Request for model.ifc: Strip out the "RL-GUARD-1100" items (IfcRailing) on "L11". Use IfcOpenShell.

First a look at what the model holds.

```python
import ifcopenshell
import ifcopenshell.util.element

model = ifcopenshell.open("model.ifc")
print(model.schema)
storey = next(s for s in model.by_type("IfcBuildingStorey") if s.Name == "L11")
railings = [e for e in ifcopenshell.util.element.get_decomposition(storey) if e.is_a("IfcRailing")]
seen = {}
for e in railings:
    element_type = ifcopenshell.util.element.get_type(e)
    name = element_type.Name if element_type not in (None, e) else None
    seen[name] = seen.get(name, 0) + 1
for name, count in sorted(seen.items(), key=str):
    print(count, "x", name)
```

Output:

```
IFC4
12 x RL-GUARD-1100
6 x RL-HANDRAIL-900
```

```python
import ifcopenshell
import ifcopenshell.api.root
import ifcopenshell.util.element

model = ifcopenshell.open("model.ifc")

storey = next(s for s in model.by_type("IfcBuildingStorey") if s.Name == "L11")
railings = [e for e in ifcopenshell.util.element.get_decomposition(storey) if e.is_a("IfcRailing")]
targets = [e for e in railings if (t := ifcopenshell.util.element.get_type(e)) not in (None, e) and t.Name == "RL-GUARD-1100"]

for e in targets:
    ifcopenshell.api.root.remove_product(model, product=e)
print(len(targets), "removed")

model.write("model_updated.ifc")
```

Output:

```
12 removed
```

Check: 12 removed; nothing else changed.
